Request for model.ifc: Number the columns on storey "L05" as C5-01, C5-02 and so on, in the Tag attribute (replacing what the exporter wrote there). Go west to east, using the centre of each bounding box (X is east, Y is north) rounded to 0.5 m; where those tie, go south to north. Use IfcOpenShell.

First a look at what the model holds.

```python
import ifcopenshell
import ifcopenshell.util.element
import ifcopenshell.util.placement

model = ifcopenshell.open("model.ifc")
print(model.schema)
storey = next(s for s in model.by_type("IfcBuildingStorey") if s.Name == "L05")
columns = [e for e in ifcopenshell.util.element.get_decomposition(storey) if e.is_a("IfcColumn")]
for e in sorted(columns, key=lambda e: e.id()):
    origin = ifcopenshell.util.placement.get_local_placement(e.ObjectPlacement)[:3, 3]
    print(e.id(), e.Tag, e.Name, origin.round(2) + 0.0, sep=" | ")
```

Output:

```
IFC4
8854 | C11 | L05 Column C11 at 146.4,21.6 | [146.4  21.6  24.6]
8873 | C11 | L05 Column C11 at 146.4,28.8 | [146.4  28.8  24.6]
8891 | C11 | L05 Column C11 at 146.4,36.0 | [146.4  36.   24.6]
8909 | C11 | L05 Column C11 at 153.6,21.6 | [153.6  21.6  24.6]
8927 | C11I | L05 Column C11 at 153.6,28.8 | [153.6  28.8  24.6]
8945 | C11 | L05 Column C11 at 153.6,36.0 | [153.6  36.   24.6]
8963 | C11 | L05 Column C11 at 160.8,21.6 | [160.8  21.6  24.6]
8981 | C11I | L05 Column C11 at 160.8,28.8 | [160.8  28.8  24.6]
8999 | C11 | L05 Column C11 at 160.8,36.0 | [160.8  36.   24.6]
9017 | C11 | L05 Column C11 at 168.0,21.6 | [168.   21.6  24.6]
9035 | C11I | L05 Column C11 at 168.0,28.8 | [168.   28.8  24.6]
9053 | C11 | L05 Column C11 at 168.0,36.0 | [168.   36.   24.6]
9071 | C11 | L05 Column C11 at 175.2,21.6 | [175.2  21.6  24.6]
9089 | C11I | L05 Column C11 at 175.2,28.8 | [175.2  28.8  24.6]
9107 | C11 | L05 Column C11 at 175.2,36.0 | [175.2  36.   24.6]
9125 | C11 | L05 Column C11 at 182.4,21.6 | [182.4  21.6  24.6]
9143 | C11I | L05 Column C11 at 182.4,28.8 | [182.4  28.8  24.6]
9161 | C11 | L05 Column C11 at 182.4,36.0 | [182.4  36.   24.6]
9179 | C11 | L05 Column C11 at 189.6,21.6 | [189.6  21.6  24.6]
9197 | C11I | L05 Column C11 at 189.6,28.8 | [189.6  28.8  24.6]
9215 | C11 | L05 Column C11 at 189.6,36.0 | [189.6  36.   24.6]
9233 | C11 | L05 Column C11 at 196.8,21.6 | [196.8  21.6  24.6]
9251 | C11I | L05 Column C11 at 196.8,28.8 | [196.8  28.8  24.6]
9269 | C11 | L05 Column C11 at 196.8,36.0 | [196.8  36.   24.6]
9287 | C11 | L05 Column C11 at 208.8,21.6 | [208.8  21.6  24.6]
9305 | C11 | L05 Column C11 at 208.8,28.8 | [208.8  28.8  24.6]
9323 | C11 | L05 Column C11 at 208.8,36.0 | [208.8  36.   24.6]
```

```python
import ifcopenshell
import ifcopenshell.geom
import ifcopenshell.util.element
import ifcopenshell.util.shape

model = ifcopenshell.open("model.ifc")
settings = ifcopenshell.geom.settings()
settings.set("use-world-coords", True)


def centre(element):
    shape = ifcopenshell.geom.create_shape(settings, element)
    return ifcopenshell.util.shape.get_bbox_centroid(shape.geometry)


storey = next(s for s in model.by_type("IfcBuildingStorey") if s.Name == "L05")
columns = [e for e in ifcopenshell.util.element.get_decomposition(storey) if e.is_a("IfcColumn")]

# Insertion points can sit at a corner or the storey origin, so sort by the geometry (in metres).
centres = {e: centre(e) for e in columns}
columns.sort(key=lambda e: (round(centres[e][0] / 0.5), centres[e][1]))

for i, e in enumerate(columns, start=1):
    number = f"C5-{i:02d}"
    e.Tag = number
    print(e.id(), number)

model.write("model_updated.ifc")
```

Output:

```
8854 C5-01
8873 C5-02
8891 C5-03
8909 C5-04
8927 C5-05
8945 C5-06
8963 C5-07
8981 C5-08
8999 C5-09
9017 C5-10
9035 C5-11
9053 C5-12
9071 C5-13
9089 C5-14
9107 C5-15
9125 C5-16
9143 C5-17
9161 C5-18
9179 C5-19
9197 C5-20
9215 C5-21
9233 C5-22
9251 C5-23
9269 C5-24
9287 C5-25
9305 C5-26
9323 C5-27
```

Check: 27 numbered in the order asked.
